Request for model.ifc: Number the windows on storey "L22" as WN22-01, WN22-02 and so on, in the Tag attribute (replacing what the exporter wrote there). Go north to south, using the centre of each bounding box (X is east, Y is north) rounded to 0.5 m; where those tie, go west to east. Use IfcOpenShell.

First a look at what the model holds.

```python
import ifcopenshell
import ifcopenshell.util.element
import ifcopenshell.util.placement

model = ifcopenshell.open("model.ifc")
print(model.schema)
storey = next(s for s in model.by_type("IfcBuildingStorey") if s.Name == "L22")
windows = [e for e in ifcopenshell.util.element.get_decomposition(storey) if e.is_a("IfcWindow")]
for e in sorted(windows, key=lambda e: e.id()):
    origin = ifcopenshell.util.placement.get_local_placement(e.ObjectPlacement)[:3, 3]
    print(e.id(), e.Tag, e.Name, origin.round(2) + 0.0, sep=" | ")
```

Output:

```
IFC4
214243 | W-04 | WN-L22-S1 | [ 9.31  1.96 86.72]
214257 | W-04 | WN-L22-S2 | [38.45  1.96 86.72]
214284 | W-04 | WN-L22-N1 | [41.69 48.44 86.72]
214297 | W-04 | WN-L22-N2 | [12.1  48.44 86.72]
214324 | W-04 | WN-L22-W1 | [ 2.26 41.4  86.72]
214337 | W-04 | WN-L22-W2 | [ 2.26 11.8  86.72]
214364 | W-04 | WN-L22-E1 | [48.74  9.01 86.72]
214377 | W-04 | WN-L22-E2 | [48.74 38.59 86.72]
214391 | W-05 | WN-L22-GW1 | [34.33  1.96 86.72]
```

```python
import ifcopenshell
import ifcopenshell.geom
import ifcopenshell.util.element
import ifcopenshell.util.shape

model = ifcopenshell.open("model.ifc")
settings = ifcopenshell.geom.settings()
settings.set("use-world-coords", True)


def centre(element):
    shape = ifcopenshell.geom.create_shape(settings, element)
    return ifcopenshell.util.shape.get_bbox_centroid(shape.geometry)


storey = next(s for s in model.by_type("IfcBuildingStorey") if s.Name == "L22")
windows = [e for e in ifcopenshell.util.element.get_decomposition(storey) if e.is_a("IfcWindow")]

# Insertion points can sit at a corner or the storey origin, so sort by the geometry (in metres).
centres = {e: centre(e) for e in windows}
windows.sort(key=lambda e: (-round(centres[e][1] / 0.5), centres[e][0]))

for i, e in enumerate(windows, start=1):
    number = f"WN22-{i:02d}"
    e.Tag = number
    print(e.id(), number)

model.write("model_v2.ifc")
```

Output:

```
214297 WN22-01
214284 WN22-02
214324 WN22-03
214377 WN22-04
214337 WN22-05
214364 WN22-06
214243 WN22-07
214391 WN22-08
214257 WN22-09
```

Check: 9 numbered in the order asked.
